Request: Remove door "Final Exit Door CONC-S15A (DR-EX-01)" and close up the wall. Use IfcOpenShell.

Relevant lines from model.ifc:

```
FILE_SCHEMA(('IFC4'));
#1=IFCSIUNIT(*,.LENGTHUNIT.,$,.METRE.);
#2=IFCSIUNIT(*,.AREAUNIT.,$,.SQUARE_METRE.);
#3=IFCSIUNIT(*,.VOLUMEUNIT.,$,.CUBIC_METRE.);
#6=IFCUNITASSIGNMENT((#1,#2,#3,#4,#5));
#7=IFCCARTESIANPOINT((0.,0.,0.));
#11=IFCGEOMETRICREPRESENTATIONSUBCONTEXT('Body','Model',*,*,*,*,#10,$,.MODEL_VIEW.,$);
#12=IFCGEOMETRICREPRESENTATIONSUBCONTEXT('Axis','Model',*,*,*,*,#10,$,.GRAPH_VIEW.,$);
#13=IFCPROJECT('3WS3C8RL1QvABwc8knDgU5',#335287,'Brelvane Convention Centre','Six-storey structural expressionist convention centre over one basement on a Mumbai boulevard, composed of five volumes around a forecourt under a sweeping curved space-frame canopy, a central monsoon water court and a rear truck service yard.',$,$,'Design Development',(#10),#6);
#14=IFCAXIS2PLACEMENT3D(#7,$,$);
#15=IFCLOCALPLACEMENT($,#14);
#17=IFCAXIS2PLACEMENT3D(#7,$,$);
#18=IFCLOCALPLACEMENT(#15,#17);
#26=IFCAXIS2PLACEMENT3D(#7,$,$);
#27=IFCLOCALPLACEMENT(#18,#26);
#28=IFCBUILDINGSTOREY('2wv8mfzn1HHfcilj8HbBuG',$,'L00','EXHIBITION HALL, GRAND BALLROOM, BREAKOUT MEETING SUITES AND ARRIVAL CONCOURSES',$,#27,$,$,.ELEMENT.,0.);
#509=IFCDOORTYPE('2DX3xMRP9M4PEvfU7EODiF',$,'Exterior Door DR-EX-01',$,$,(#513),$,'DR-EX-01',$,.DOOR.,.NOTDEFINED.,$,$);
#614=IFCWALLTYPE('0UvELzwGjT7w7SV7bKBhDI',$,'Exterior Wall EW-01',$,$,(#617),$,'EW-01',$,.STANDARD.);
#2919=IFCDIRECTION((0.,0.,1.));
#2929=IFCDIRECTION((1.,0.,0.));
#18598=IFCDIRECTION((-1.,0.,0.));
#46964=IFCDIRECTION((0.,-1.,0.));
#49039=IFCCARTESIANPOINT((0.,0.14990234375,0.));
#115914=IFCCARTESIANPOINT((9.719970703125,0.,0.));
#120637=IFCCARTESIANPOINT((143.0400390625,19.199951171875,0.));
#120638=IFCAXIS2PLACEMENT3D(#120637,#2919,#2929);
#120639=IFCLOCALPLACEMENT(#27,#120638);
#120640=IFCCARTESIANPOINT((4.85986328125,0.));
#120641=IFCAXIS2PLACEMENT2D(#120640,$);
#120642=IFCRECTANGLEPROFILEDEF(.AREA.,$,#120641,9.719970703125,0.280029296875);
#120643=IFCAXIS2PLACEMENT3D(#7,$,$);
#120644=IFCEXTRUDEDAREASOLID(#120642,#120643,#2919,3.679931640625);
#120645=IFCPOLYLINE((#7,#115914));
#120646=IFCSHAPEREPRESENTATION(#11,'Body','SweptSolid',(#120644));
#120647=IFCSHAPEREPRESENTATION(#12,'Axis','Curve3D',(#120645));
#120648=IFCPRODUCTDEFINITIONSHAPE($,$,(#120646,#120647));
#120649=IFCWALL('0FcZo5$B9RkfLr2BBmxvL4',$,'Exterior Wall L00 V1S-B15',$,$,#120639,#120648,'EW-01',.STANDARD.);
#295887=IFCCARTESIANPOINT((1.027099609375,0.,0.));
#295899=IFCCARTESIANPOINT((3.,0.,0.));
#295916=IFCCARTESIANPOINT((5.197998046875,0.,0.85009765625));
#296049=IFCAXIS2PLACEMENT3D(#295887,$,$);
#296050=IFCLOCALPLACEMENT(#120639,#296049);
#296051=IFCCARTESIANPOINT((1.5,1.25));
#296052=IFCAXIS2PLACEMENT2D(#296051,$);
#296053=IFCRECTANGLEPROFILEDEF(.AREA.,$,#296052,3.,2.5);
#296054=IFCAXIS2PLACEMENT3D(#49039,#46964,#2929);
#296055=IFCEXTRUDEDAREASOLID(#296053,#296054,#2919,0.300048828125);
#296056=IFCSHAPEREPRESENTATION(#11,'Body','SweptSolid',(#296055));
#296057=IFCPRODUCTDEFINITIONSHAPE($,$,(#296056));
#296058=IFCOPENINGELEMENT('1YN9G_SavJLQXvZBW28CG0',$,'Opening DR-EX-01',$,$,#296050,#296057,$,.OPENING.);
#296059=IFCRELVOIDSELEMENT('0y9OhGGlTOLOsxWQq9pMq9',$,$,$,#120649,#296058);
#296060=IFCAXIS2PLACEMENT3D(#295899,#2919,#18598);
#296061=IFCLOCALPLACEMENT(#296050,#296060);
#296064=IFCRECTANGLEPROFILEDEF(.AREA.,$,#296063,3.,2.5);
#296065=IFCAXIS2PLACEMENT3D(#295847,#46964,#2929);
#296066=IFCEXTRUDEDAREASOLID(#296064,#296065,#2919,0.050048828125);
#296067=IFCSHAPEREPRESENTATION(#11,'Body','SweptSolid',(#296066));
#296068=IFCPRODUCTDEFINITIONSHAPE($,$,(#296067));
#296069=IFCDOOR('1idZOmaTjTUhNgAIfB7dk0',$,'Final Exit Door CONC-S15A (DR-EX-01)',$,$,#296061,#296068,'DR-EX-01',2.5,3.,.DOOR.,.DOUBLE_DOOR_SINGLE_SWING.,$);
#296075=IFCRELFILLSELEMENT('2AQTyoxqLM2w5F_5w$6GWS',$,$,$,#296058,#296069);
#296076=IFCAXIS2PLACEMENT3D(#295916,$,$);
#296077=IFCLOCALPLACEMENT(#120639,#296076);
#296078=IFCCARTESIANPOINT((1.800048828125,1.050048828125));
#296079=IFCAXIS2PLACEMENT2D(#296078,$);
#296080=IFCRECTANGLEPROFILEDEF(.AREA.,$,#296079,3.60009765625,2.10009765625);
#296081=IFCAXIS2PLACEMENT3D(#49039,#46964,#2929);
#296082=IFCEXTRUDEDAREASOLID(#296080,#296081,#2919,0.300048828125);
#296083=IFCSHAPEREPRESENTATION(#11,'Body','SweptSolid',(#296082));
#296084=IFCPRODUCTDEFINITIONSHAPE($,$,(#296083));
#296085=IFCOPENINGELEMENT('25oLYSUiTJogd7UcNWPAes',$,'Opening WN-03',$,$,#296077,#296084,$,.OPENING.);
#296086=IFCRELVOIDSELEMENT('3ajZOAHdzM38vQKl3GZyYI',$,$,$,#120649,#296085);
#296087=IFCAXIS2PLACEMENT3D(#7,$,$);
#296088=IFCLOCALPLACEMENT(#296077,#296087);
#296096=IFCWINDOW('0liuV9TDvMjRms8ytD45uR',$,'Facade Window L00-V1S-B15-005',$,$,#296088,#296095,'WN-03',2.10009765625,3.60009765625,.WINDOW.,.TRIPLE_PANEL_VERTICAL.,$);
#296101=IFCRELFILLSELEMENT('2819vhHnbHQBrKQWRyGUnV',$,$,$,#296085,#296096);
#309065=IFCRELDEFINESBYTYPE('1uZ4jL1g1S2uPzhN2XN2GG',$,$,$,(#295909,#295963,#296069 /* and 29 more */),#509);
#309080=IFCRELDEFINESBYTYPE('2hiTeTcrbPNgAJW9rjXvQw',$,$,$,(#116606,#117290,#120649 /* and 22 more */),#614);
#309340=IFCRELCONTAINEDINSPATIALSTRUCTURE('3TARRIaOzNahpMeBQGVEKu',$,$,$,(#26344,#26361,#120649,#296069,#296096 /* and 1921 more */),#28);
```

```python
import ifcopenshell
import ifcopenshell.api.feature
import ifcopenshell.api.root
import ifcopenshell.geom
import ifcopenshell.util.shape

model = ifcopenshell.open("model.ifc")
settings = ifcopenshell.geom.settings()


def volume(element):
    """Net volume in cubic metres, openings subtracted."""
    shape = ifcopenshell.geom.create_shape(settings, element)
    return ifcopenshell.util.shape.get_volume(shape.geometry)


door = model.by_guid("1idZOmaTjTUhNgAIfB7dk0")
opening = door.FillsVoids[0].RelatingOpeningElement
wall = opening.VoidsElements[0].RelatingBuildingElement
before = volume(wall)

ifcopenshell.api.root.remove_product(model, product=door)
ifcopenshell.api.feature.remove_feature(model, feature=opening)

after = volume(wall)

print(f"wall volume {before:.3f} -> {after:.3f} m3")

model.write("model_edited.ifc")
```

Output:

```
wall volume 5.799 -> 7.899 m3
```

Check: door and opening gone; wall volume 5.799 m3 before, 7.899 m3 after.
